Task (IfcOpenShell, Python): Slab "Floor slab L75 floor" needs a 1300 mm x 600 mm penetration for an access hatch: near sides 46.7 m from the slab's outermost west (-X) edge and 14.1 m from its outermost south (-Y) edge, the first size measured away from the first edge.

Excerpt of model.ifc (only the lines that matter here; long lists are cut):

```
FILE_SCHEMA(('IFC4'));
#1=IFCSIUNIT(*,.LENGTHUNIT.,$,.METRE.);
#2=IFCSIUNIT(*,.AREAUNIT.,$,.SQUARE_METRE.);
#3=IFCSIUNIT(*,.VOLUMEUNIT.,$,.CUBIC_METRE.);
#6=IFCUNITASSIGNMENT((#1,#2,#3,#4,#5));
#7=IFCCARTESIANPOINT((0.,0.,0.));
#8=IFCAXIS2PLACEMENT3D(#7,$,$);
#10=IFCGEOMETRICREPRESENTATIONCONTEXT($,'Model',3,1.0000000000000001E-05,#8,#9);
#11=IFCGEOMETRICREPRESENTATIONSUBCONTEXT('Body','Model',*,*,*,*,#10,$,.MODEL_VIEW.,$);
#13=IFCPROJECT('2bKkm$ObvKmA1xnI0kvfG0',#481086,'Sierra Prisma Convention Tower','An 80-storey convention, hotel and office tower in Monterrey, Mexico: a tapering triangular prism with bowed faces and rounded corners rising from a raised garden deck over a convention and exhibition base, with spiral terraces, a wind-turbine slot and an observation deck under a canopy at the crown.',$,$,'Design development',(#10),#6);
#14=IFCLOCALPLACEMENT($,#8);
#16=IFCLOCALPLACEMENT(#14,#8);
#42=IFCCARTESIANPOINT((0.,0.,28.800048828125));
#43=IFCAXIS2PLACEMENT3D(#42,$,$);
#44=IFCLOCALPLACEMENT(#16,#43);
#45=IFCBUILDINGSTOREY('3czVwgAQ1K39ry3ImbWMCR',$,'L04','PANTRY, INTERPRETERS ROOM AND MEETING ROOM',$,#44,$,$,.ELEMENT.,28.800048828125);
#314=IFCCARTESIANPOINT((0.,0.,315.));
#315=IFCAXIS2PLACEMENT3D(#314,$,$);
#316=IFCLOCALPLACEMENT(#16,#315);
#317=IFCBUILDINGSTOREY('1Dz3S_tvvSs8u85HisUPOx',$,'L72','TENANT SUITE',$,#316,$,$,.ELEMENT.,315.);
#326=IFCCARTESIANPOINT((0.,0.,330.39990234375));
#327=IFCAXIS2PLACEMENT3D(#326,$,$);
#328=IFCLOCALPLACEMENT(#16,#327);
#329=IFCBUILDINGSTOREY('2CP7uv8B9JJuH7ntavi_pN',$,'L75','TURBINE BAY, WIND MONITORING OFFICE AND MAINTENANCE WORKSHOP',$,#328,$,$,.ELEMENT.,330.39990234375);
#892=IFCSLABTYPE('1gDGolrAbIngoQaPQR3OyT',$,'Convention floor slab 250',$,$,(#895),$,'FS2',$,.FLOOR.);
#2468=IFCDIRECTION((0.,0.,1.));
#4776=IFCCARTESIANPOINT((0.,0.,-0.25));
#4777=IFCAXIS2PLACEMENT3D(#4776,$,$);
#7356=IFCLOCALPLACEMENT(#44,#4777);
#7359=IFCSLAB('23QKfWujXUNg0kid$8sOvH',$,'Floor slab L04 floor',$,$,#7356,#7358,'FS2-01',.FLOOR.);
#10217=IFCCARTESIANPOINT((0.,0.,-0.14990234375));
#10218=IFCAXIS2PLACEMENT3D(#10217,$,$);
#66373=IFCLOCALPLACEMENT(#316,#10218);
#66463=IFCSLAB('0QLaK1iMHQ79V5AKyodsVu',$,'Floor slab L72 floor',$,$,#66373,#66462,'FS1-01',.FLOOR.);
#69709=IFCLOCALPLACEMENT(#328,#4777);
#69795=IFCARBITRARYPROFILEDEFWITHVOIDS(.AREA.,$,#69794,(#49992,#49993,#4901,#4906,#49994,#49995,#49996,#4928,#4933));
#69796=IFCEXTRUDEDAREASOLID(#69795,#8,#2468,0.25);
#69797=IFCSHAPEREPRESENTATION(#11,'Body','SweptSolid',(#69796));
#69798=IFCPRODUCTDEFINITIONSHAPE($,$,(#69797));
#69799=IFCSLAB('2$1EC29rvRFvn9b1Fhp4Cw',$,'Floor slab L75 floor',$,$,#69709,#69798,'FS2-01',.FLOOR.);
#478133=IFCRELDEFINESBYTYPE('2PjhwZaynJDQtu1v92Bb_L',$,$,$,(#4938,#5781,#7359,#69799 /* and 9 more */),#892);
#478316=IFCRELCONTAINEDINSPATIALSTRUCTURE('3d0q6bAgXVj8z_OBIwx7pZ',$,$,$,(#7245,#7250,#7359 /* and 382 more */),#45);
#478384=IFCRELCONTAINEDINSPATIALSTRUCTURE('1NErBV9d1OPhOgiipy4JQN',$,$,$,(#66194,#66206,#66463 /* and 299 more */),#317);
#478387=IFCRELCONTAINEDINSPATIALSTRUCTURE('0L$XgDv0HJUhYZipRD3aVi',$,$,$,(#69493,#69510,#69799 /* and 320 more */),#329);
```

```python
import numpy as np
import ifcopenshell
import ifcopenshell.api.feature
import ifcopenshell.api.geometry
import ifcopenshell.api.root
import ifcopenshell.geom
import ifcopenshell.util.placement
import ifcopenshell.util.representation
import ifcopenshell.util.shape
import ifcopenshell.util.unit

model = ifcopenshell.open("model.ifc")
unit_scale = ifcopenshell.util.unit.calculate_unit_scale(model)
settings = ifcopenshell.geom.settings()


def volume(element):
    """Net volume in cubic metres, openings subtracted."""
    shape = ifcopenshell.geom.create_shape(settings, element)
    return ifcopenshell.util.shape.get_volume(shape.geometry)


slab = model.by_guid("2$1EC29rvRFvn9b1Fhp4Cw")
before = volume(slab)

# Extent in the slab's own axes, in metres. The edges named are its -X and -Y sides.
slab_shape = ifcopenshell.geom.create_shape(settings, slab)
vertices = ifcopenshell.util.shape.get_vertices(slab_shape.geometry)
x_min, y_min, bottom = vertices.min(axis=0)
top = vertices[:, 2].max()

opening = ifcopenshell.api.root.create_entity(model, ifc_class="IfcOpeningElement", name="Access hatch opening", predefined_type="OPENING")
context = ifcopenshell.util.representation.get_context(model, "Model", "Body", "MODEL_VIEW")
width, depth = 1.3, 0.6
outline = [(0.0, 0.0), (width, 0.0), (width, depth), (0.0, depth), (0.0, 0.0)]
# Overshoot both faces by 50 mm so the cut is clean.
shape = ifcopenshell.api.geometry.add_slab_representation(
    model, context=context, depth=top - bottom + 0.1, polyline=outline
)
ifcopenshell.api.geometry.assign_representation(model, product=opening, representation=shape)

matrix = ifcopenshell.util.placement.get_local_placement(slab.ObjectPlacement)
matrix[:, 3] = matrix @ np.append(np.array([x_min + 46.7, y_min + 14.1, bottom - 0.05]) / unit_scale, 1.0)
ifcopenshell.api.geometry.edit_object_placement(model, product=opening, matrix=matrix, is_si=False)
ifcopenshell.api.feature.add_feature(model, feature=opening, element=slab)

after = volume(slab)

print(f"slab volume {before:.3f} -> {after:.3f} m3")

model.write("model_edited.ifc")
```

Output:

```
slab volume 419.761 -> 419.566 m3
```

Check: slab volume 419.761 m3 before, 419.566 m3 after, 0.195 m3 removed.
